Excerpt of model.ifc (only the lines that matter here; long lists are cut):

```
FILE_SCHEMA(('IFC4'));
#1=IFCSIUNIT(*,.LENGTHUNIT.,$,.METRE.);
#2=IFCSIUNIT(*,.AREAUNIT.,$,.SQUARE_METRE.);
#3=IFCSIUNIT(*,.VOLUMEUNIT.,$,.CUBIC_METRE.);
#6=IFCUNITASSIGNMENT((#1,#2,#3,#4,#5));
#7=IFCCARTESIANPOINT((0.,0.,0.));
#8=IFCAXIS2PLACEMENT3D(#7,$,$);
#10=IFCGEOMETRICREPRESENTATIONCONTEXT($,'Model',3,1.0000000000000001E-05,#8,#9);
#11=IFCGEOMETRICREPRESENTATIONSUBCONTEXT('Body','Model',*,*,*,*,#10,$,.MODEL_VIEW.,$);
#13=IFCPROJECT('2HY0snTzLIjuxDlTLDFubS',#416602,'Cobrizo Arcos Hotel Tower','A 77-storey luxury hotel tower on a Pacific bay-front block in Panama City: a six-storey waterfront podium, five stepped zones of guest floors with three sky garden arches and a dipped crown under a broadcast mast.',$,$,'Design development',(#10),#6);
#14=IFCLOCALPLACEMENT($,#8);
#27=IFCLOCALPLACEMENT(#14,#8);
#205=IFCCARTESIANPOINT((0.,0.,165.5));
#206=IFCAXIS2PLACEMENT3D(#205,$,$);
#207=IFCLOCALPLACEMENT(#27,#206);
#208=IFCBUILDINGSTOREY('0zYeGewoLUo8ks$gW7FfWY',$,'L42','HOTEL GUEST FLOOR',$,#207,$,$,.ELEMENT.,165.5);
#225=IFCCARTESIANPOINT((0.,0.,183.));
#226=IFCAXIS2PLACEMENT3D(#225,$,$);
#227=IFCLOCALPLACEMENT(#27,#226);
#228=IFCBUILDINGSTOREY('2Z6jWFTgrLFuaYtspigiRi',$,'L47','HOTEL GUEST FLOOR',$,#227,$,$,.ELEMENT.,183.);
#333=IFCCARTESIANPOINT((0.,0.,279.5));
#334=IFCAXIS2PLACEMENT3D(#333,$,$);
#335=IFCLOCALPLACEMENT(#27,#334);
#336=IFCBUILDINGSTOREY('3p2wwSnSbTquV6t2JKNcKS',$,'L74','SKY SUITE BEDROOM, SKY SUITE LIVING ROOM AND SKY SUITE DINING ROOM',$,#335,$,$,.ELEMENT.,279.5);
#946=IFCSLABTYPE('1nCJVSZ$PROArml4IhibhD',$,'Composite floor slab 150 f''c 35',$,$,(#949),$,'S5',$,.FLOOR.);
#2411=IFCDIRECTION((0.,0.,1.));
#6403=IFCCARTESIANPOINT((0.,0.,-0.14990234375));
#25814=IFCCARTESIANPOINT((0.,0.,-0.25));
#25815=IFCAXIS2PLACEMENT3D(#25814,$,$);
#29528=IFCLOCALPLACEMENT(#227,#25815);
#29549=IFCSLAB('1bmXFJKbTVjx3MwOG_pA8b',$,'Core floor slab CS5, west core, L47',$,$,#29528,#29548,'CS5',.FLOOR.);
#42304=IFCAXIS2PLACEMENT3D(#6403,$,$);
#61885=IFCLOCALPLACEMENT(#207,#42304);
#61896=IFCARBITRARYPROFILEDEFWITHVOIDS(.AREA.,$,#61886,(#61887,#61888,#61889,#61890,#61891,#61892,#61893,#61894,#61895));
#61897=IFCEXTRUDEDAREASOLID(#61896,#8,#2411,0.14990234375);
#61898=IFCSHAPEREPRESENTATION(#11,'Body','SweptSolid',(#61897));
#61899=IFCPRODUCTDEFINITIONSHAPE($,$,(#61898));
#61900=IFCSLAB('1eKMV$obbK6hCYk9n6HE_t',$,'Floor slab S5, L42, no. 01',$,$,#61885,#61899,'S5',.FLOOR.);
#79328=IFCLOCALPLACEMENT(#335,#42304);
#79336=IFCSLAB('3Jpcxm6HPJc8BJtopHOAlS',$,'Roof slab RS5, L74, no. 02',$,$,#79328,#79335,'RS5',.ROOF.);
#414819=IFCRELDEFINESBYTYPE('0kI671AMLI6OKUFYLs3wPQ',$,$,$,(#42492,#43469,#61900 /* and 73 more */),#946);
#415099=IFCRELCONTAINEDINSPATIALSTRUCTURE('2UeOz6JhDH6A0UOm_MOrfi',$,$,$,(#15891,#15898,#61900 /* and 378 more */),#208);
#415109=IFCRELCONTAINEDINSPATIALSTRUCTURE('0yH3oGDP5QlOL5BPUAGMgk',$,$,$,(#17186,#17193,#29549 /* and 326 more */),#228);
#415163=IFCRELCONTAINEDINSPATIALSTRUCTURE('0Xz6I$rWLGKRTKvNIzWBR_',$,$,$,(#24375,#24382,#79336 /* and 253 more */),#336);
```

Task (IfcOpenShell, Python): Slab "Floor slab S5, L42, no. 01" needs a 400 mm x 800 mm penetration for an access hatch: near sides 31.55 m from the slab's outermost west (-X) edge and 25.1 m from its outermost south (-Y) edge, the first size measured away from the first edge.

```python
import numpy as np
import ifcopenshell
import ifcopenshell.api.feature
import ifcopenshell.api.geometry
import ifcopenshell.api.root
import ifcopenshell.geom
import ifcopenshell.util.placement
import ifcopenshell.util.representation
import ifcopenshell.util.shape
import ifcopenshell.util.unit

model = ifcopenshell.open("model.ifc")
unit_scale = ifcopenshell.util.unit.calculate_unit_scale(model)
settings = ifcopenshell.geom.settings()


def volume(element):
    """Net volume in cubic metres, openings subtracted."""
    shape = ifcopenshell.geom.create_shape(settings, element)
    return ifcopenshell.util.shape.get_volume(shape.geometry)


slab = model.by_id(61900)
before = volume(slab)

# Extent in the slab's own axes, in metres. The edges named are its -X and -Y sides.
slab_shape = ifcopenshell.geom.create_shape(settings, slab)
vertices = ifcopenshell.util.shape.get_vertices(slab_shape.geometry)
x_min, y_min, bottom = vertices.min(axis=0)
top = vertices[:, 2].max()

opening = ifcopenshell.api.root.create_entity(model, ifc_class="IfcOpeningElement", name="Access hatch opening", predefined_type="OPENING")
context = ifcopenshell.util.representation.get_context(model, "Model", "Body", "MODEL_VIEW")
width, depth = 0.4, 0.8
outline = [(0.0, 0.0), (width, 0.0), (width, depth), (0.0, depth), (0.0, 0.0)]
# Overshoot both faces by 50 mm so the cut is clean.
shape = ifcopenshell.api.geometry.add_slab_representation(
    model, context=context, depth=top - bottom + 0.1, polyline=outline
)
ifcopenshell.api.geometry.assign_representation(model, product=opening, representation=shape)

matrix = ifcopenshell.util.placement.get_local_placement(slab.ObjectPlacement)
matrix[:, 3] = matrix @ np.append(np.array([x_min + 31.55, y_min + 25.1, bottom - 0.05]) / unit_scale, 1.0)
ifcopenshell.api.geometry.edit_object_placement(model, product=opening, matrix=matrix, is_si=False)
ifcopenshell.api.feature.add_feature(model, feature=opening, element=slab)

after = volume(slab)

print(f"slab volume {before:.3f} -> {after:.3f} m3")

model.write("model-out.ifc")
```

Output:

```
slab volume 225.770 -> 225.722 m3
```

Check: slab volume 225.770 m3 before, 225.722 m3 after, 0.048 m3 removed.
